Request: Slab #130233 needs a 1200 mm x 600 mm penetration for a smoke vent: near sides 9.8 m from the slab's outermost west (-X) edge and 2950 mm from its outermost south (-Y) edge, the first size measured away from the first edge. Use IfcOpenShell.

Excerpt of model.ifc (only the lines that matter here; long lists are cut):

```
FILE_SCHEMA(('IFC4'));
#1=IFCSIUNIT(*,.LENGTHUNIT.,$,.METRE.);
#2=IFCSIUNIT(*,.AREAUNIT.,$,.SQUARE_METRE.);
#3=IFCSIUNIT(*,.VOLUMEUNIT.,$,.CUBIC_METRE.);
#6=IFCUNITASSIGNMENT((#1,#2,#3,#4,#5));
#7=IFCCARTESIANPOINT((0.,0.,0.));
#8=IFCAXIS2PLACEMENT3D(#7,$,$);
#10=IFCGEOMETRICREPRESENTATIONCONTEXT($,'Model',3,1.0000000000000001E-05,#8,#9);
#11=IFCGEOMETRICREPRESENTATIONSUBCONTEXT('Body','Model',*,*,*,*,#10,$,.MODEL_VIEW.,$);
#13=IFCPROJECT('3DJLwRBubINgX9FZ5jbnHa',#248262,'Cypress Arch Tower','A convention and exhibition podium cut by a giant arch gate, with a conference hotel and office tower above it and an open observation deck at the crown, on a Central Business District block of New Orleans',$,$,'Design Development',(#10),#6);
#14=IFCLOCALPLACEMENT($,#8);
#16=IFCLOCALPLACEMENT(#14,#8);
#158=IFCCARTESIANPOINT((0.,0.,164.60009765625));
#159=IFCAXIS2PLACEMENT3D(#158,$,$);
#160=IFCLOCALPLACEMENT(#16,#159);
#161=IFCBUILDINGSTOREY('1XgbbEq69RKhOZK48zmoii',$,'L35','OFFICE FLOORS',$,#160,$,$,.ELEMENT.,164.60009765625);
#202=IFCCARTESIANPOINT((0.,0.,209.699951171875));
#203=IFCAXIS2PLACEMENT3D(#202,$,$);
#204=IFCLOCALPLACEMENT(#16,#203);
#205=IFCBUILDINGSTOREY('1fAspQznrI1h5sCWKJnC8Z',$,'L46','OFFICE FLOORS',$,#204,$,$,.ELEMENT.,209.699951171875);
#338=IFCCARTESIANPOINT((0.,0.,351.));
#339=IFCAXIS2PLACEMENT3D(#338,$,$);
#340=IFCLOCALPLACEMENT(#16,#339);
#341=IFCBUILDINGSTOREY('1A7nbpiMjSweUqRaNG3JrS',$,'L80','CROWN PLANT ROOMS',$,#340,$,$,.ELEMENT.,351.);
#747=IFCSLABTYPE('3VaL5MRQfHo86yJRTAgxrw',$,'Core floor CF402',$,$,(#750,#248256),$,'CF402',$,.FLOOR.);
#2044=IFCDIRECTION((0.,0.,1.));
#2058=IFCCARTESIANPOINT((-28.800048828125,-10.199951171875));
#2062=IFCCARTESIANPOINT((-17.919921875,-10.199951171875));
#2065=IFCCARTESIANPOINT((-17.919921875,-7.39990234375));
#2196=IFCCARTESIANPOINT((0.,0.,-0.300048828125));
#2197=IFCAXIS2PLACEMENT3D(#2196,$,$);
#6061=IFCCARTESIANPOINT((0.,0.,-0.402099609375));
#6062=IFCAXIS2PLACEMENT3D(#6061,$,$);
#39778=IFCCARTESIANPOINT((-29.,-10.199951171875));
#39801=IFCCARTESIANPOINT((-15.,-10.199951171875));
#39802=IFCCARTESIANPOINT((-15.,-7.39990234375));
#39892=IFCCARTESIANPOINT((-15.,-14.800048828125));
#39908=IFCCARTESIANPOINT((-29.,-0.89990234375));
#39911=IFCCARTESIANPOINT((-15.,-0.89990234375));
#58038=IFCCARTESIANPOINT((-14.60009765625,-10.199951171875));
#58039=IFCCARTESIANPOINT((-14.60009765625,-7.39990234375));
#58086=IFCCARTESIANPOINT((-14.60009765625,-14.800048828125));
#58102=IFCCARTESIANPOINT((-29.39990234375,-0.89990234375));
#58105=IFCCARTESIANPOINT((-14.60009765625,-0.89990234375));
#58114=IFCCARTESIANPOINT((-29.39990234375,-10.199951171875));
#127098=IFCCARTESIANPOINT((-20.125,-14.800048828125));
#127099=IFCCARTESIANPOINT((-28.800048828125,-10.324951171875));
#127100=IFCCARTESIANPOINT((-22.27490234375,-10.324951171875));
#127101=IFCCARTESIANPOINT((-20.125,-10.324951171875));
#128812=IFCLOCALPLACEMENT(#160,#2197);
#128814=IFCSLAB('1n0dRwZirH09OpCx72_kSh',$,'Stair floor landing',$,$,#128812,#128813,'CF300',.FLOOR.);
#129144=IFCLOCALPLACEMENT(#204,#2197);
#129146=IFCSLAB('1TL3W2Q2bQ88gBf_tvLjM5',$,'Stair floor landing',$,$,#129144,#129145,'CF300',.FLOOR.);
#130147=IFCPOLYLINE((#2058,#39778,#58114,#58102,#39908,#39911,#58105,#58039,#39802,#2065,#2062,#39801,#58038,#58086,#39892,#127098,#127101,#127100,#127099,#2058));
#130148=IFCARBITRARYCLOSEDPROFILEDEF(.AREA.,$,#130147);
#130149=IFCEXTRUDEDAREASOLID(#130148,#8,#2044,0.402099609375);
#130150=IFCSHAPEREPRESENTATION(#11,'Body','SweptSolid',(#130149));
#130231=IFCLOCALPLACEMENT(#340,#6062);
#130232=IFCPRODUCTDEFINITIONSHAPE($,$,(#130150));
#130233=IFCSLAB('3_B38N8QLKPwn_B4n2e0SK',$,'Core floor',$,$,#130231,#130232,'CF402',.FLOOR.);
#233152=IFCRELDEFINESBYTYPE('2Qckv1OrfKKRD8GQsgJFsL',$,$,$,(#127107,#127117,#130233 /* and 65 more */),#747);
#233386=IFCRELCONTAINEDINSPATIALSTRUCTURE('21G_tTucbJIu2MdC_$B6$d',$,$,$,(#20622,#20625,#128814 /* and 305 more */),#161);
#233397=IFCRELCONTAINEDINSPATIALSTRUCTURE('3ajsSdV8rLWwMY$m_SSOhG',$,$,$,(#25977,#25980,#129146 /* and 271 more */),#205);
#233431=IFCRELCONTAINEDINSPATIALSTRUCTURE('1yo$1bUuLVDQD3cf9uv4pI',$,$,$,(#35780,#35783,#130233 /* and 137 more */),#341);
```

```python
import numpy as np
import ifcopenshell
import ifcopenshell.api.feature
import ifcopenshell.api.geometry
import ifcopenshell.api.root
import ifcopenshell.geom
import ifcopenshell.util.placement
import ifcopenshell.util.representation
import ifcopenshell.util.shape
import ifcopenshell.util.unit

model = ifcopenshell.open("model.ifc")
unit_scale = ifcopenshell.util.unit.calculate_unit_scale(model)
settings = ifcopenshell.geom.settings()


def volume(element):
    """Net volume in cubic metres, openings subtracted."""
    shape = ifcopenshell.geom.create_shape(settings, element)
    return ifcopenshell.util.shape.get_volume(shape.geometry)


slab = model.by_guid("3_B38N8QLKPwn_B4n2e0SK")
before = volume(slab)

# Extent in the slab's own axes, in metres. The edges named are its -X and -Y sides.
slab_shape = ifcopenshell.geom.create_shape(settings, slab)
vertices = ifcopenshell.util.shape.get_vertices(slab_shape.geometry)
x_min, y_min, bottom = vertices.min(axis=0)
top = vertices[:, 2].max()

opening = ifcopenshell.api.root.create_entity(model, ifc_class="IfcOpeningElement", name="Smoke vent opening", predefined_type="OPENING")
context = ifcopenshell.util.representation.get_context(model, "Model", "Body", "MODEL_VIEW")
width, depth = 1.2, 0.6
outline = [(0.0, 0.0), (width, 0.0), (width, depth), (0.0, depth), (0.0, 0.0)]
# Overshoot both faces by 50 mm so the cut is clean.
shape = ifcopenshell.api.geometry.add_slab_representation(
    model, context=context, depth=top - bottom + 0.1, polyline=outline
)
ifcopenshell.api.geometry.assign_representation(model, product=opening, representation=shape)

matrix = ifcopenshell.util.placement.get_local_placement(slab.ObjectPlacement)
matrix[:, 3] = matrix @ np.append(np.array([x_min + 9.8, y_min + 2.95, bottom - 0.05]) / unit_scale, 1.0)
ifcopenshell.api.geometry.edit_object_placement(model, product=opening, matrix=matrix, is_si=False)
ifcopenshell.api.feature.add_feature(model, feature=opening, element=slab)

after = volume(slab)

print(f"slab volume {before:.3f} -> {after:.3f} m3")

model.write("model-out.ifc")
```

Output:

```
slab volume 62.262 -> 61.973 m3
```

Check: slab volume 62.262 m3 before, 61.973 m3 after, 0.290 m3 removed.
